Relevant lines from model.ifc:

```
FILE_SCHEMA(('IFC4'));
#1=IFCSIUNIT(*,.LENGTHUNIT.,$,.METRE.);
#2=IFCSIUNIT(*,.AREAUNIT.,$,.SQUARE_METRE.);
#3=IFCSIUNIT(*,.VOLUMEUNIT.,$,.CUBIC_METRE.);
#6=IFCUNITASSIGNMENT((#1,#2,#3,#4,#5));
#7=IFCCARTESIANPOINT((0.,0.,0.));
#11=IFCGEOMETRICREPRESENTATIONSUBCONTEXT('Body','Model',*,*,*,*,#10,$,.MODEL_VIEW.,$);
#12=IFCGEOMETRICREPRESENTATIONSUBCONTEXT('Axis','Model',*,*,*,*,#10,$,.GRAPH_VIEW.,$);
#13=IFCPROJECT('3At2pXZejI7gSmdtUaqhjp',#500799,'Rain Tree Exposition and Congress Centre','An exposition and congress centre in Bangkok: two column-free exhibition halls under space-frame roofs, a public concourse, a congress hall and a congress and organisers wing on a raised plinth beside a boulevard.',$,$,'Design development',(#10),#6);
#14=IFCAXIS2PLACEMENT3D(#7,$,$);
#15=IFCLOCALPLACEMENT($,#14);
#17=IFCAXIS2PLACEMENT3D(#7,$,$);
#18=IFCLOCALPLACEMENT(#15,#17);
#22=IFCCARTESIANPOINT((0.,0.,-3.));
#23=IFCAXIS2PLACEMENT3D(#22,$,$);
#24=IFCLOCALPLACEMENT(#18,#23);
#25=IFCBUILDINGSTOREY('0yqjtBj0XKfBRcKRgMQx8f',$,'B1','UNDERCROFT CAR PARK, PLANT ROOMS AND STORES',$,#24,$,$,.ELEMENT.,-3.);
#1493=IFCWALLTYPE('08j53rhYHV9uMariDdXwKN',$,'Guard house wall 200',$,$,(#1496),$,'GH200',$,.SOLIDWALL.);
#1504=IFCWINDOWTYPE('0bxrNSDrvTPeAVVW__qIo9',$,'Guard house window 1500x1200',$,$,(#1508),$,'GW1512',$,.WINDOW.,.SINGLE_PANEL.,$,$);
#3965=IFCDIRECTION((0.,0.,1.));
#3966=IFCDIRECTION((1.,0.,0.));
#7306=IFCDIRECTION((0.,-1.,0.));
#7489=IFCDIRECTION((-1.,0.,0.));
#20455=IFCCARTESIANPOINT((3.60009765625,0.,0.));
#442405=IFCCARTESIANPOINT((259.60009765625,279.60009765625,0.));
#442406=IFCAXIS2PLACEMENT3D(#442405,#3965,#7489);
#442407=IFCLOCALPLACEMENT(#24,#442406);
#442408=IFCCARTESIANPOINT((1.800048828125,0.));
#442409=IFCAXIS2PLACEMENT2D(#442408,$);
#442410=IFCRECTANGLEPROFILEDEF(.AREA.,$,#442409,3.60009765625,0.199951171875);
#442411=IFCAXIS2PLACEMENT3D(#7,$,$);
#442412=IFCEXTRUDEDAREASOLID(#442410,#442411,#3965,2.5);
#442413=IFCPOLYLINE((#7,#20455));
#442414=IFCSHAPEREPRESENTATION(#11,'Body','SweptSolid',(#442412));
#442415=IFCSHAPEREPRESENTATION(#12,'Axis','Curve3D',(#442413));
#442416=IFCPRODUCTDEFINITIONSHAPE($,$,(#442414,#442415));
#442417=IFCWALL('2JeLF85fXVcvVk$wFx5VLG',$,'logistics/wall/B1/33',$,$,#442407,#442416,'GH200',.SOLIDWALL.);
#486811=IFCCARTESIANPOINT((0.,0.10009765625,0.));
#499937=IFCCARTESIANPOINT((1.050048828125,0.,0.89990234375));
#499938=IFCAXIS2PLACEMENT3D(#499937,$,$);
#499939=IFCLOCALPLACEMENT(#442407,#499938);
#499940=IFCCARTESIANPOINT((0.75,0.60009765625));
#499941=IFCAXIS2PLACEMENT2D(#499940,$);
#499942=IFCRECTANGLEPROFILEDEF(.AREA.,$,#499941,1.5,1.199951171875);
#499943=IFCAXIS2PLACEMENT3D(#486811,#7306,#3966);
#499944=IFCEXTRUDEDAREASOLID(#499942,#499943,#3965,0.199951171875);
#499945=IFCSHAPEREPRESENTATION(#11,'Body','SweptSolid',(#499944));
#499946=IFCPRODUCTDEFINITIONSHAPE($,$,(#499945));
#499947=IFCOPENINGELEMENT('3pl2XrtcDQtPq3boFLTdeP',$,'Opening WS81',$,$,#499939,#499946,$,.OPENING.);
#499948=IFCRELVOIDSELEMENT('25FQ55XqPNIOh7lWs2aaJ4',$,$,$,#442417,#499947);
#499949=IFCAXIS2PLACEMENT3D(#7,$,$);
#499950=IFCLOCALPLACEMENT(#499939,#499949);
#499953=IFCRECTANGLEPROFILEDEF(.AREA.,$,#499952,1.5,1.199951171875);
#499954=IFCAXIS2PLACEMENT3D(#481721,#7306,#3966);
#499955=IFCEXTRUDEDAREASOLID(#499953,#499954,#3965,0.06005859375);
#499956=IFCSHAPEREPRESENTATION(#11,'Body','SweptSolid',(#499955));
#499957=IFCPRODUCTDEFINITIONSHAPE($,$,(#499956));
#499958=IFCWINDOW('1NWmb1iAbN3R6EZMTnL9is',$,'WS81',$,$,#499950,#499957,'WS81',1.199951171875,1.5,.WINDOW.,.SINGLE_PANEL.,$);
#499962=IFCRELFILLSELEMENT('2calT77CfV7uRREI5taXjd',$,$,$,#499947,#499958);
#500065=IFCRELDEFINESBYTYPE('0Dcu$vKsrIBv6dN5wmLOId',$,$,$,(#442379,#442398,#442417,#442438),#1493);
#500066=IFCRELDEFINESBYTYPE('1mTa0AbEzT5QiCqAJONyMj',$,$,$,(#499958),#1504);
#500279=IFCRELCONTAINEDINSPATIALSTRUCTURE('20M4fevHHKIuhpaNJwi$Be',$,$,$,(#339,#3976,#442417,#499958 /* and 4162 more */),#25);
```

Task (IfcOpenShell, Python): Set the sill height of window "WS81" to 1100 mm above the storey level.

```python
import numpy as np
import ifcopenshell
import ifcopenshell.api.geometry
import ifcopenshell.geom
import ifcopenshell.util.element
import ifcopenshell.util.placement
import ifcopenshell.util.shape
import ifcopenshell.util.unit

model = ifcopenshell.open("model.ifc")
unit_scale = ifcopenshell.util.unit.calculate_unit_scale(model)

window = model.by_guid("1NWmb1iAbN3R6EZMTnL9is")
opening = window.FillsVoids[0].RelatingOpeningElement
storey = ifcopenshell.util.element.get_container(window, ifc_class="IfcBuildingStorey")
level = ifcopenshell.util.placement.get_local_placement(storey.ObjectPlacement)[2, 3]

# The opening's origin need not be at the sill, so measure its lowest point.
shape = ifcopenshell.geom.create_shape(ifcopenshell.geom.settings(), opening)
bottom = ifcopenshell.util.shape.get_shape_bottom_elevation(shape, shape.geometry) / unit_scale
dz = level + 1.1 - bottom

shift = np.array([0.0, 0.0, dz])
# The window is placed relative to its opening, so it follows when the opening moves.
matrix = ifcopenshell.util.placement.get_local_placement(opening.ObjectPlacement)
matrix[:3, 3] += shift
ifcopenshell.api.geometry.edit_object_placement(
    model, product=opening, matrix=matrix, is_si=False, should_transform_children=True
)

print(f"moved by {dz * unit_scale:+.3f} m")

model.write("model_edited.ifc")
```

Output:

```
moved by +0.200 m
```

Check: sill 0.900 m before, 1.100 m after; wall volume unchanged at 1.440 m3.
